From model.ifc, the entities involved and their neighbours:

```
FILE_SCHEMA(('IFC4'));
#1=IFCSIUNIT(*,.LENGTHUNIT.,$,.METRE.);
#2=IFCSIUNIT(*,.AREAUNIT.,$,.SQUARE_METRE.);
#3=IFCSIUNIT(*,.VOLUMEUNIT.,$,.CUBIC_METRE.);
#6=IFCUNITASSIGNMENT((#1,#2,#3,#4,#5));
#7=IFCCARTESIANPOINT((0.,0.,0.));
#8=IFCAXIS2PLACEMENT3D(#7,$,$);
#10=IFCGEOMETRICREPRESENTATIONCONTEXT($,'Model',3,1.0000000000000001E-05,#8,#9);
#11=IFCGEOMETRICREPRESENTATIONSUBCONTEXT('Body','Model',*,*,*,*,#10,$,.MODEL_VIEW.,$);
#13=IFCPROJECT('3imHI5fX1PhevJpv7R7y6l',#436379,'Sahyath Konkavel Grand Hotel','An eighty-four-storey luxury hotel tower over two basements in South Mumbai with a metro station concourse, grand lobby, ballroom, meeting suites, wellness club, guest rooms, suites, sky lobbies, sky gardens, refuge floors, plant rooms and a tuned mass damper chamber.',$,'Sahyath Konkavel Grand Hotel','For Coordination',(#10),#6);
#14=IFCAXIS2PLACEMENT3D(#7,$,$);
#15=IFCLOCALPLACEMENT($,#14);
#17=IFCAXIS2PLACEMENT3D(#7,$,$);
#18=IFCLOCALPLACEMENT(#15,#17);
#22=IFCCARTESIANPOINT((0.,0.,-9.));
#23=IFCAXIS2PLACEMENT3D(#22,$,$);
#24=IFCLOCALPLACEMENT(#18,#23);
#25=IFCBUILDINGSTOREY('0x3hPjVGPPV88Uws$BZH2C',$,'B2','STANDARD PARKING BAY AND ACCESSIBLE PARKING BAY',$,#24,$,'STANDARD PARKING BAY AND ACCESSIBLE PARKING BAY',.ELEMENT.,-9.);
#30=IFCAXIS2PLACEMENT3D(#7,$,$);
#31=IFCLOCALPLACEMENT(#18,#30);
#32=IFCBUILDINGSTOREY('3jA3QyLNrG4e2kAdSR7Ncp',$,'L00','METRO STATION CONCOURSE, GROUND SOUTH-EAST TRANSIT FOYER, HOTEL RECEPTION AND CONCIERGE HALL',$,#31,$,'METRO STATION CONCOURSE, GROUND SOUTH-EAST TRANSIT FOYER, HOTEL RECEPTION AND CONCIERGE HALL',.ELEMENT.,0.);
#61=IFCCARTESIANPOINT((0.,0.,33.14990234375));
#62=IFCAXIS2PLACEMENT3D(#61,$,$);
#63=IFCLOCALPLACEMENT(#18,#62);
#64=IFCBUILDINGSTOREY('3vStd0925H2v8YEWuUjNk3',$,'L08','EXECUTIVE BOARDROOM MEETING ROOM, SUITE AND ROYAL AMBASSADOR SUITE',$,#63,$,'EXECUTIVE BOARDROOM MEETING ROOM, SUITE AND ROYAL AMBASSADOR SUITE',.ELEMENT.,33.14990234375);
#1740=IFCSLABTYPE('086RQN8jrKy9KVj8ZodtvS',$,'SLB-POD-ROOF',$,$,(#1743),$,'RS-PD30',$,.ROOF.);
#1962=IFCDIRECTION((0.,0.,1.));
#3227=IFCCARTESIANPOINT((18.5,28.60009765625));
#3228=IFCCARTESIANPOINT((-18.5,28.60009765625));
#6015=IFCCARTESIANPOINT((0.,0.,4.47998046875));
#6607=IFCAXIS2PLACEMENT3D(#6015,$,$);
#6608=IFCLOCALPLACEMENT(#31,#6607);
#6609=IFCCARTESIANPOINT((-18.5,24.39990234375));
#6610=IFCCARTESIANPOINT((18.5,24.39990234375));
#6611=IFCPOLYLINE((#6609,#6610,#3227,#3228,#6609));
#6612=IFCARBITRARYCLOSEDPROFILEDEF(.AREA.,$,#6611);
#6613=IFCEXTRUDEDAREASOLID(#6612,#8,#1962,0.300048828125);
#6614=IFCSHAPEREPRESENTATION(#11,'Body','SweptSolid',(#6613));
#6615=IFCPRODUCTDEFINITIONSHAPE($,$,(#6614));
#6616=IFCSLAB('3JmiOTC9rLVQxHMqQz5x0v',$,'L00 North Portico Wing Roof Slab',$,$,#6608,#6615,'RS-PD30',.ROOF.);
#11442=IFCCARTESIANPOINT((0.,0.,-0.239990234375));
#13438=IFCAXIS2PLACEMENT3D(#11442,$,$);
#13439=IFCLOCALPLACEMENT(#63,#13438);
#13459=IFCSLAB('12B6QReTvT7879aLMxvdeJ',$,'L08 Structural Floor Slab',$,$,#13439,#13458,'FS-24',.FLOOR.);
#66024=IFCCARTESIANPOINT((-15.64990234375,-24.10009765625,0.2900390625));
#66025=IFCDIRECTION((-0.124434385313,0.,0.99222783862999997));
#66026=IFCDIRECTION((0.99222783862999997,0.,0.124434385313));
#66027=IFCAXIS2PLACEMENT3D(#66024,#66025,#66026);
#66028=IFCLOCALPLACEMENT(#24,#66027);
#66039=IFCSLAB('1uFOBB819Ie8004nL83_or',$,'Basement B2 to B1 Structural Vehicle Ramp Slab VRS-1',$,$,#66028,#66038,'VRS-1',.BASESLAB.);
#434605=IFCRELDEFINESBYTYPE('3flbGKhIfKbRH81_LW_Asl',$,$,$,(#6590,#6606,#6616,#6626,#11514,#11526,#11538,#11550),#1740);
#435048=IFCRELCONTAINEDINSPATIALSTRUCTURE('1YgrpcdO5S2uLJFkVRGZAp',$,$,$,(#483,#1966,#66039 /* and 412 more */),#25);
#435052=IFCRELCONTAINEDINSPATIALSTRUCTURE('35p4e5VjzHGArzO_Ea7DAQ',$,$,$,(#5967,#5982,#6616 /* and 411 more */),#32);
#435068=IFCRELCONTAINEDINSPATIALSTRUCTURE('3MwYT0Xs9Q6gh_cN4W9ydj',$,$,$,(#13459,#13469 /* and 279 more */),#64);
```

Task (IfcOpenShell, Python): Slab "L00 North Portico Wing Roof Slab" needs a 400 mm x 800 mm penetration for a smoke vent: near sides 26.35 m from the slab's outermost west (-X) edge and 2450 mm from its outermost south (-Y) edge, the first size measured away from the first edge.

```python
import numpy as np
import ifcopenshell
import ifcopenshell.api.feature
import ifcopenshell.api.geometry
import ifcopenshell.api.root
import ifcopenshell.geom
import ifcopenshell.util.placement
import ifcopenshell.util.representation
import ifcopenshell.util.shape
import ifcopenshell.util.unit

model = ifcopenshell.open("model.ifc")
unit_scale = ifcopenshell.util.unit.calculate_unit_scale(model)
settings = ifcopenshell.geom.settings()


def volume(element):
    """Net volume in cubic metres, openings subtracted."""
    shape = ifcopenshell.geom.create_shape(settings, element)
    return ifcopenshell.util.shape.get_volume(shape.geometry)


slab = model.by_guid("3JmiOTC9rLVQxHMqQz5x0v")
before = volume(slab)

# Extent in the slab's own axes, in metres. The edges named are its -X and -Y sides.
slab_shape = ifcopenshell.geom.create_shape(settings, slab)
vertices = ifcopenshell.util.shape.get_vertices(slab_shape.geometry)
x_min, y_min, bottom = vertices.min(axis=0)
top = vertices[:, 2].max()

opening = ifcopenshell.api.root.create_entity(model, ifc_class="IfcOpeningElement", name="Smoke vent opening", predefined_type="OPENING")
context = ifcopenshell.util.representation.get_context(model, "Model", "Body", "MODEL_VIEW")
width, depth = 0.4, 0.8
outline = [(0.0, 0.0), (width, 0.0), (width, depth), (0.0, depth), (0.0, 0.0)]
# Overshoot both faces by 50 mm so the cut is clean.
shape = ifcopenshell.api.geometry.add_slab_representation(
    model, context=context, depth=top - bottom + 0.1, polyline=outline
)
ifcopenshell.api.geometry.assign_representation(model, product=opening, representation=shape)

matrix = ifcopenshell.util.placement.get_local_placement(slab.ObjectPlacement)
matrix[:, 3] = matrix @ np.append(np.array([x_min + 26.35, y_min + 2.45, bottom - 0.05]) / unit_scale, 1.0)
ifcopenshell.api.geometry.edit_object_placement(model, product=opening, matrix=matrix, is_si=False)
ifcopenshell.api.feature.add_feature(model, feature=opening, element=slab)

after = volume(slab)

print(f"slab volume {before:.3f} -> {after:.3f} m3")

model.write("model_updated.ifc")
```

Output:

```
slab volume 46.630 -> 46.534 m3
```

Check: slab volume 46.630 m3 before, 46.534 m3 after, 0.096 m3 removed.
